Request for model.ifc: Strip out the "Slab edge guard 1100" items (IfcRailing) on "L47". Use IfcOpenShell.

First a look at what the model holds.

```python
import ifcopenshell
import ifcopenshell.util.element

model = ifcopenshell.open("model.ifc")
print(model.schema)
storey = next(s for s in model.by_type("IfcBuildingStorey") if s.Name == "L47")
railings = [e for e in ifcopenshell.util.element.get_decomposition(storey) if e.is_a("IfcRailing")]
seen = {}
for e in railings:
    element_type = ifcopenshell.util.element.get_type(e)
    name = element_type.Name if element_type not in (None, e) else None
    seen[name] = seen.get(name, 0) + 1
for name, count in sorted(seen.items(), key=str):
    print(count, "x", name)
```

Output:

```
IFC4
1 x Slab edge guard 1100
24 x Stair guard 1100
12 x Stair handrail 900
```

```python
import ifcopenshell
import ifcopenshell.api.root
import ifcopenshell.util.element

model = ifcopenshell.open("model.ifc")

storey = next(s for s in model.by_type("IfcBuildingStorey") if s.Name == "L47")
railings = [e for e in ifcopenshell.util.element.get_decomposition(storey) if e.is_a("IfcRailing")]
targets = [e for e in railings if (t := ifcopenshell.util.element.get_type(e)) not in (None, e) and t.Name == "Slab edge guard 1100"]

for e in targets:
    ifcopenshell.api.root.remove_product(model, product=e)
print(len(targets), "removed")

model.write("model-out.ifc")
```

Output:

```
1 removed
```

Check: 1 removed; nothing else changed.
